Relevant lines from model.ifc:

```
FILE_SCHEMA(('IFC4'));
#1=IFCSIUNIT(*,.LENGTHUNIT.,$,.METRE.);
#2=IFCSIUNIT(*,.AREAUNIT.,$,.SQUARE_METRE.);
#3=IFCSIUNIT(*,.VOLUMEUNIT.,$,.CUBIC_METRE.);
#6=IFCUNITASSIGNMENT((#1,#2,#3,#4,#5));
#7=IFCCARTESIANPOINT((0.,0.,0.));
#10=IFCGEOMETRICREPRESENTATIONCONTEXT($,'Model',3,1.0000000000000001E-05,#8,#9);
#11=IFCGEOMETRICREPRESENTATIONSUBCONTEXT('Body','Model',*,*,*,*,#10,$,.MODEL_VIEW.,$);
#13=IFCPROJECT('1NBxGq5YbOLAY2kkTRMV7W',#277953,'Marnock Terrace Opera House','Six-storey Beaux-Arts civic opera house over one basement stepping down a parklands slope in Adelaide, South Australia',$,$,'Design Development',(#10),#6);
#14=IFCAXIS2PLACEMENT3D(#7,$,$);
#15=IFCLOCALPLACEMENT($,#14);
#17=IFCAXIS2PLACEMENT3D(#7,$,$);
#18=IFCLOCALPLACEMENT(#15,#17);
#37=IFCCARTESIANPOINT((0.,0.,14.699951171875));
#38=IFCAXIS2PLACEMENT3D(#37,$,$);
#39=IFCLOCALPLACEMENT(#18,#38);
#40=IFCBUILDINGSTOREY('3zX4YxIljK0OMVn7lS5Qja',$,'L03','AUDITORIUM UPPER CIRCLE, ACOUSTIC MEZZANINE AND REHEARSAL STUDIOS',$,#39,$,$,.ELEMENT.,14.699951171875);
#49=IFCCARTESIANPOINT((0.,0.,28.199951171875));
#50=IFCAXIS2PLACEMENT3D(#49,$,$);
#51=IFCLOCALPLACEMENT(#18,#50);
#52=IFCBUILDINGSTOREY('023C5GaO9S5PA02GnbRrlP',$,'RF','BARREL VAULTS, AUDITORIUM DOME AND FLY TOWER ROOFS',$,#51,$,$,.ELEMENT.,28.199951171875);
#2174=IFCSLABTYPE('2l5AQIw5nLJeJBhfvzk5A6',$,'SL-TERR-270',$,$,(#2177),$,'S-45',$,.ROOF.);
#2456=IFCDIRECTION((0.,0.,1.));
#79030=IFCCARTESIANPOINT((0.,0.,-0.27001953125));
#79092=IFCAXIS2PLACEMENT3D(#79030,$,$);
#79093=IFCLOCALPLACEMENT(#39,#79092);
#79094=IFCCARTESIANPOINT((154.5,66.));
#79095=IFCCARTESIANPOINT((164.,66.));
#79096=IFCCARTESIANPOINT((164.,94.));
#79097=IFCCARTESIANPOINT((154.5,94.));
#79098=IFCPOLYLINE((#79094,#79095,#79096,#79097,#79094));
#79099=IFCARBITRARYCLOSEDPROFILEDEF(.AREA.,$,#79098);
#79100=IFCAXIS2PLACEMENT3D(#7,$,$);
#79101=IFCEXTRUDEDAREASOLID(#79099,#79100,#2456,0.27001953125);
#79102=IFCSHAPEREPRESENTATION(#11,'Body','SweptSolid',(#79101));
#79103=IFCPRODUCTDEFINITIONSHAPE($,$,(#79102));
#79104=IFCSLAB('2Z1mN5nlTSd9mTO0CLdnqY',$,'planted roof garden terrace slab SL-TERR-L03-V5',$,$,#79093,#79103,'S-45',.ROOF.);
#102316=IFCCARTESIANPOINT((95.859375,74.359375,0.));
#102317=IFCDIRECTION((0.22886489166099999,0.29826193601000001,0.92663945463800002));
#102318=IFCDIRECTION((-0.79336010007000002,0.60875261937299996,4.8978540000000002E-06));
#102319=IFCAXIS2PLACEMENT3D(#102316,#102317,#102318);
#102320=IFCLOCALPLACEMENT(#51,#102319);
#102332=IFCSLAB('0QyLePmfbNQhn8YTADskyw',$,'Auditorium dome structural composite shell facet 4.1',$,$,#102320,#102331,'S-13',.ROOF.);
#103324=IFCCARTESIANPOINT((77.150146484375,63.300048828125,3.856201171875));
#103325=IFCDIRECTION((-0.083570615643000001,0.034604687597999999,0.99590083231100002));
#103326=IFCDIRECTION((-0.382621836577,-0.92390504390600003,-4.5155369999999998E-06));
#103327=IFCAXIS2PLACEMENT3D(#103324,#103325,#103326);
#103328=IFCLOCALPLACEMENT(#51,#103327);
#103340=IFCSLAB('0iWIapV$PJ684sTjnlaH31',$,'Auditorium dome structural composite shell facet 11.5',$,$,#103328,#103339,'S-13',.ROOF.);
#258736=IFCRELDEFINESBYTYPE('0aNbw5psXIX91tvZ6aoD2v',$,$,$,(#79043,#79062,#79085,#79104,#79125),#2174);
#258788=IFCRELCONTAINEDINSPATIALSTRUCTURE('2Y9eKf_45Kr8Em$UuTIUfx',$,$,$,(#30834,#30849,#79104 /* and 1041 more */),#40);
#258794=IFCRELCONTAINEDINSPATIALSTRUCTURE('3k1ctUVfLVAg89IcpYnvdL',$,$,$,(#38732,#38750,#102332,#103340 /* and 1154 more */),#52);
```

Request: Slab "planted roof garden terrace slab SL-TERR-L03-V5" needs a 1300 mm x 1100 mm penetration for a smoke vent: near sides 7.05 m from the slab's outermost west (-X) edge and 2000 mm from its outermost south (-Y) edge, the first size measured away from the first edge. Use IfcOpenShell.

```python
import numpy as np
import ifcopenshell
import ifcopenshell.api.feature
import ifcopenshell.api.geometry
import ifcopenshell.api.root
import ifcopenshell.geom
import ifcopenshell.util.placement
import ifcopenshell.util.representation
import ifcopenshell.util.shape
import ifcopenshell.util.unit

model = ifcopenshell.open("model.ifc")
unit_scale = ifcopenshell.util.unit.calculate_unit_scale(model)
settings = ifcopenshell.geom.settings()


def volume(element):
    """Net volume in cubic metres, openings subtracted."""
    shape = ifcopenshell.geom.create_shape(settings, element)
    return ifcopenshell.util.shape.get_volume(shape.geometry)


slab = model.by_guid("2Z1mN5nlTSd9mTO0CLdnqY")
before = volume(slab)

# Extent in the slab's own axes, in metres. The edges named are its -X and -Y sides.
slab_shape = ifcopenshell.geom.create_shape(settings, slab)
vertices = ifcopenshell.util.shape.get_vertices(slab_shape.geometry)
x_min, y_min, bottom = vertices.min(axis=0)
top = vertices[:, 2].max()

opening = ifcopenshell.api.root.create_entity(model, ifc_class="IfcOpeningElement", name="Smoke vent opening", predefined_type="OPENING")
context = ifcopenshell.util.representation.get_context(model, "Model", "Body", "MODEL_VIEW")
width, depth = 1.3, 1.1
outline = [(0.0, 0.0), (width, 0.0), (width, depth), (0.0, depth), (0.0, 0.0)]
# Overshoot both faces by 50 mm so the cut is clean.
shape = ifcopenshell.api.geometry.add_slab_representation(
    model, context=context, depth=top - bottom + 0.1, polyline=outline
)
ifcopenshell.api.geometry.assign_representation(model, product=opening, representation=shape)

matrix = ifcopenshell.util.placement.get_local_placement(slab.ObjectPlacement)
matrix[:, 3] = matrix @ np.append(np.array([x_min + 7.05, y_min + 2, bottom - 0.05]) / unit_scale, 1.0)
ifcopenshell.api.geometry.edit_object_placement(model, product=opening, matrix=matrix, is_si=False)
ifcopenshell.api.feature.add_feature(model, feature=opening, element=slab)

after = volume(slab)

print(f"slab volume {before:.3f} -> {after:.3f} m3")

model.write("model_updated.ifc")
```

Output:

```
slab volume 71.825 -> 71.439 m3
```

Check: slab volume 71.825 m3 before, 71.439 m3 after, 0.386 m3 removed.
